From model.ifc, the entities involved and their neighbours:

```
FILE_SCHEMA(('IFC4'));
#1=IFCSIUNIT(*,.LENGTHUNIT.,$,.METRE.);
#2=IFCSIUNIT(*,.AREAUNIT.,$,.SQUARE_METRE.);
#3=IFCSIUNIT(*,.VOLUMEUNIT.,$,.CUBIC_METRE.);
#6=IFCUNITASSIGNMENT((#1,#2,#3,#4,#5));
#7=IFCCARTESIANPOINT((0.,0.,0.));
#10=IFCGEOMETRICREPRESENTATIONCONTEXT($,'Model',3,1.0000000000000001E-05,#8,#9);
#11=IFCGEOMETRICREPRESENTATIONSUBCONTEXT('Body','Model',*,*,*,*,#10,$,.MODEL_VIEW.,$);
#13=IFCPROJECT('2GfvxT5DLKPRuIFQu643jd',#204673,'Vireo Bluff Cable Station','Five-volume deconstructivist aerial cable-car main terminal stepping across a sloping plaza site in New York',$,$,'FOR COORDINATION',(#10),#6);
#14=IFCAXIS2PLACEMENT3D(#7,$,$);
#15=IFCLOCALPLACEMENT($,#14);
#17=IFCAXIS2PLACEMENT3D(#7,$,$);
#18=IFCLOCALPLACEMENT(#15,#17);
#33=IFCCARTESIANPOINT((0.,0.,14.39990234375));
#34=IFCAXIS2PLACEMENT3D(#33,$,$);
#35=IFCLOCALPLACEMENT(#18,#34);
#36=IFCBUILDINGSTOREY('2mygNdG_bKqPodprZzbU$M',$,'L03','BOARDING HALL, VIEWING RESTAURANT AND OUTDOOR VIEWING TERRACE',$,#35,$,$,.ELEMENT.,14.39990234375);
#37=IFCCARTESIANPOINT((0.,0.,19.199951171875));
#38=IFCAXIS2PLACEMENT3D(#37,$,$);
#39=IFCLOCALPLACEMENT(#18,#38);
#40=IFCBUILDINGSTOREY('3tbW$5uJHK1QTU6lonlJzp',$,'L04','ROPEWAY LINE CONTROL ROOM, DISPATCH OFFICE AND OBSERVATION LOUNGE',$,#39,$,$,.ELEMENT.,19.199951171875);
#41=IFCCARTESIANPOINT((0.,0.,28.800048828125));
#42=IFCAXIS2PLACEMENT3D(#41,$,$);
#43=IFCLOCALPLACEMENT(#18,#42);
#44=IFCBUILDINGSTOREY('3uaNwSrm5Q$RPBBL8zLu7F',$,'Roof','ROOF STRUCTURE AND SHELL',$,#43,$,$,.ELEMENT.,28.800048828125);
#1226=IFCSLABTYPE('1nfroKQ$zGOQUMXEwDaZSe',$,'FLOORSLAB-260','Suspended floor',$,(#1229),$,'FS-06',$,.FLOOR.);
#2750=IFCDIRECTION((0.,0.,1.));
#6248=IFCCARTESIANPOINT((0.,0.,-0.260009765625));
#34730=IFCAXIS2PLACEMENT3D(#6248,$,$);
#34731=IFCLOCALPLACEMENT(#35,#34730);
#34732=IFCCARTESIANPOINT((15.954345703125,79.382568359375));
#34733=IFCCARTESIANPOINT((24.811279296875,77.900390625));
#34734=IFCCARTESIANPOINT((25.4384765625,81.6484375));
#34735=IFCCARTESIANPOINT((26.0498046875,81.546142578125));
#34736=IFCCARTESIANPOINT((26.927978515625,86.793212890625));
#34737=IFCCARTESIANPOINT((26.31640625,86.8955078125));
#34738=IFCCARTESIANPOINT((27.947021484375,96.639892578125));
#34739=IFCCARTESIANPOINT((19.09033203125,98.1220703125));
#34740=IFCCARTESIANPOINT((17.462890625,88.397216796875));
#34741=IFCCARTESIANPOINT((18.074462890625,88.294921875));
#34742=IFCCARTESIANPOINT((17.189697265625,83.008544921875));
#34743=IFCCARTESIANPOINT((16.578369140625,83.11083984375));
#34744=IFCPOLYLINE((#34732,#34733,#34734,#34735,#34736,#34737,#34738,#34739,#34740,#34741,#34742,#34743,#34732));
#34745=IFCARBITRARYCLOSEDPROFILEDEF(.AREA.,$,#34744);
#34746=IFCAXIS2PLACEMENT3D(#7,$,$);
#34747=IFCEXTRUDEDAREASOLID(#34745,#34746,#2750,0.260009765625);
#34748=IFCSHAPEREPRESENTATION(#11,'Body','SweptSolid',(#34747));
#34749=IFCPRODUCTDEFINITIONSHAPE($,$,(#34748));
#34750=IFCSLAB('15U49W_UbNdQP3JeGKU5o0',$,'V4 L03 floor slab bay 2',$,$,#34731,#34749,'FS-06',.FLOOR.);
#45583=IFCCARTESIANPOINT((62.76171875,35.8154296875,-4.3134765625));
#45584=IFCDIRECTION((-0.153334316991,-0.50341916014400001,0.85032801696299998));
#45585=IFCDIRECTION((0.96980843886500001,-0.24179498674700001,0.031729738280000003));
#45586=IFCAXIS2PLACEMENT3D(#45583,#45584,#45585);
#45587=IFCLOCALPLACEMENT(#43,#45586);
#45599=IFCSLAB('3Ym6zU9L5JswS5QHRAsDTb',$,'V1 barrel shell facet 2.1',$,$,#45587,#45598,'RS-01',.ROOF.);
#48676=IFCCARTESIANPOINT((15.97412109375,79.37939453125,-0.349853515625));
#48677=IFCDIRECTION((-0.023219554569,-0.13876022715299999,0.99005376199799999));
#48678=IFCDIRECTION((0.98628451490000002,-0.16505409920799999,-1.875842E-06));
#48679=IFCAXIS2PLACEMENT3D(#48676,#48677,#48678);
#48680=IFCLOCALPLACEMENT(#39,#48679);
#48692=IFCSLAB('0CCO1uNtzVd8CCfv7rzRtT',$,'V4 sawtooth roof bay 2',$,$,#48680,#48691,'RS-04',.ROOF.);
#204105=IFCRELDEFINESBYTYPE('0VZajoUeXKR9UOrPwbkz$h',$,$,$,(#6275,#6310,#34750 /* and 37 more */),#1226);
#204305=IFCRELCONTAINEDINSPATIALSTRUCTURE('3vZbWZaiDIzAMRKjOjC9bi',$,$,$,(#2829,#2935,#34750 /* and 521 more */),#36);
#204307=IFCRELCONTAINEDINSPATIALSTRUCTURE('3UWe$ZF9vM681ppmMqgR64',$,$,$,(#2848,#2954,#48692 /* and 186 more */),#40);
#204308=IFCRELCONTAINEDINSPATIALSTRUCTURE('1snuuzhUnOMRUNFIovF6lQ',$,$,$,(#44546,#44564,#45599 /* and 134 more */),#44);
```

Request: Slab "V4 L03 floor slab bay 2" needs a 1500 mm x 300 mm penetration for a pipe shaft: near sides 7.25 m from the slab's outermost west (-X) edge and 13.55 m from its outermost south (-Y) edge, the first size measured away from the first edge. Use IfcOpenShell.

```python
import numpy as np
import ifcopenshell
import ifcopenshell.api.feature
import ifcopenshell.api.geometry
import ifcopenshell.api.root
import ifcopenshell.geom
import ifcopenshell.util.placement
import ifcopenshell.util.representation
import ifcopenshell.util.shape
import ifcopenshell.util.unit

model = ifcopenshell.open("model.ifc")
unit_scale = ifcopenshell.util.unit.calculate_unit_scale(model)
settings = ifcopenshell.geom.settings()


def volume(element):
    """Net volume in cubic metres, openings subtracted."""
    shape = ifcopenshell.geom.create_shape(settings, element)
    return ifcopenshell.util.shape.get_volume(shape.geometry)


slab = model.by_guid("15U49W_UbNdQP3JeGKU5o0")
before = volume(slab)

# Extent in the slab's own axes, in metres. The edges named are its -X and -Y sides.
slab_shape = ifcopenshell.geom.create_shape(settings, slab)
vertices = ifcopenshell.util.shape.get_vertices(slab_shape.geometry)
x_min, y_min, bottom = vertices.min(axis=0)
top = vertices[:, 2].max()

opening = ifcopenshell.api.root.create_entity(model, ifc_class="IfcOpeningElement", name="Pipe shaft opening", predefined_type="OPENING")
context = ifcopenshell.util.representation.get_context(model, "Model", "Body", "MODEL_VIEW")
width, depth = 1.5, 0.3
outline = [(0.0, 0.0), (width, 0.0), (width, depth), (0.0, depth), (0.0, 0.0)]
# Overshoot both faces by 50 mm so the cut is clean.
shape = ifcopenshell.api.geometry.add_slab_representation(
    model, context=context, depth=top - bottom + 0.1, polyline=outline
)
ifcopenshell.api.geometry.assign_representation(model, product=opening, representation=shape)

matrix = ifcopenshell.util.placement.get_local_placement(slab.ObjectPlacement)
matrix[:, 3] = matrix @ np.append(np.array([x_min + 7.25, y_min + 13.55, bottom - 0.05]) / unit_scale, 1.0)
ifcopenshell.api.geometry.edit_object_placement(model, product=opening, matrix=matrix, is_si=False)
ifcopenshell.api.feature.add_feature(model, feature=opening, element=slab)

after = volume(slab)

print(f"slab volume {before:.3f} -> {after:.3f} m3")

model.write("model-out.ifc")
```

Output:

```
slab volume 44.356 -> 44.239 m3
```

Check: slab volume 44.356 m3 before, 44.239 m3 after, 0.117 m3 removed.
